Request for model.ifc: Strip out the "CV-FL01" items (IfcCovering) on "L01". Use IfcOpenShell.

First a look at what the model holds.

```python
import ifcopenshell
import ifcopenshell.util.element

model = ifcopenshell.open("model.ifc")
print(model.schema)
storey = next(s for s in model.by_type("IfcBuildingStorey") if s.Name == "L01")
coverings = [e for e in ifcopenshell.util.element.get_decomposition(storey) if e.is_a("IfcCovering")]
seen = {}
for e in coverings:
    element_type = ifcopenshell.util.element.get_type(e)
    name = element_type.Name if element_type not in (None, e) else None
    seen[name] = seen.get(name, 0) + 1
for name, count in sorted(seen.items(), key=str):
    print(count, "x", name)
```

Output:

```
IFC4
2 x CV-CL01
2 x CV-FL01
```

```python
import ifcopenshell
import ifcopenshell.api.root
import ifcopenshell.util.element

model = ifcopenshell.open("model.ifc")

storey = next(s for s in model.by_type("IfcBuildingStorey") if s.Name == "L01")
coverings = [e for e in ifcopenshell.util.element.get_decomposition(storey) if e.is_a("IfcCovering")]
targets = [e for e in coverings if (t := ifcopenshell.util.element.get_type(e)) not in (None, e) and t.Name == "CV-FL01"]

for e in targets:
    ifcopenshell.api.root.remove_product(model, product=e)
print(len(targets), "removed")

model.write("model_v2.ifc")
```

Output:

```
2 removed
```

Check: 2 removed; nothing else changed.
